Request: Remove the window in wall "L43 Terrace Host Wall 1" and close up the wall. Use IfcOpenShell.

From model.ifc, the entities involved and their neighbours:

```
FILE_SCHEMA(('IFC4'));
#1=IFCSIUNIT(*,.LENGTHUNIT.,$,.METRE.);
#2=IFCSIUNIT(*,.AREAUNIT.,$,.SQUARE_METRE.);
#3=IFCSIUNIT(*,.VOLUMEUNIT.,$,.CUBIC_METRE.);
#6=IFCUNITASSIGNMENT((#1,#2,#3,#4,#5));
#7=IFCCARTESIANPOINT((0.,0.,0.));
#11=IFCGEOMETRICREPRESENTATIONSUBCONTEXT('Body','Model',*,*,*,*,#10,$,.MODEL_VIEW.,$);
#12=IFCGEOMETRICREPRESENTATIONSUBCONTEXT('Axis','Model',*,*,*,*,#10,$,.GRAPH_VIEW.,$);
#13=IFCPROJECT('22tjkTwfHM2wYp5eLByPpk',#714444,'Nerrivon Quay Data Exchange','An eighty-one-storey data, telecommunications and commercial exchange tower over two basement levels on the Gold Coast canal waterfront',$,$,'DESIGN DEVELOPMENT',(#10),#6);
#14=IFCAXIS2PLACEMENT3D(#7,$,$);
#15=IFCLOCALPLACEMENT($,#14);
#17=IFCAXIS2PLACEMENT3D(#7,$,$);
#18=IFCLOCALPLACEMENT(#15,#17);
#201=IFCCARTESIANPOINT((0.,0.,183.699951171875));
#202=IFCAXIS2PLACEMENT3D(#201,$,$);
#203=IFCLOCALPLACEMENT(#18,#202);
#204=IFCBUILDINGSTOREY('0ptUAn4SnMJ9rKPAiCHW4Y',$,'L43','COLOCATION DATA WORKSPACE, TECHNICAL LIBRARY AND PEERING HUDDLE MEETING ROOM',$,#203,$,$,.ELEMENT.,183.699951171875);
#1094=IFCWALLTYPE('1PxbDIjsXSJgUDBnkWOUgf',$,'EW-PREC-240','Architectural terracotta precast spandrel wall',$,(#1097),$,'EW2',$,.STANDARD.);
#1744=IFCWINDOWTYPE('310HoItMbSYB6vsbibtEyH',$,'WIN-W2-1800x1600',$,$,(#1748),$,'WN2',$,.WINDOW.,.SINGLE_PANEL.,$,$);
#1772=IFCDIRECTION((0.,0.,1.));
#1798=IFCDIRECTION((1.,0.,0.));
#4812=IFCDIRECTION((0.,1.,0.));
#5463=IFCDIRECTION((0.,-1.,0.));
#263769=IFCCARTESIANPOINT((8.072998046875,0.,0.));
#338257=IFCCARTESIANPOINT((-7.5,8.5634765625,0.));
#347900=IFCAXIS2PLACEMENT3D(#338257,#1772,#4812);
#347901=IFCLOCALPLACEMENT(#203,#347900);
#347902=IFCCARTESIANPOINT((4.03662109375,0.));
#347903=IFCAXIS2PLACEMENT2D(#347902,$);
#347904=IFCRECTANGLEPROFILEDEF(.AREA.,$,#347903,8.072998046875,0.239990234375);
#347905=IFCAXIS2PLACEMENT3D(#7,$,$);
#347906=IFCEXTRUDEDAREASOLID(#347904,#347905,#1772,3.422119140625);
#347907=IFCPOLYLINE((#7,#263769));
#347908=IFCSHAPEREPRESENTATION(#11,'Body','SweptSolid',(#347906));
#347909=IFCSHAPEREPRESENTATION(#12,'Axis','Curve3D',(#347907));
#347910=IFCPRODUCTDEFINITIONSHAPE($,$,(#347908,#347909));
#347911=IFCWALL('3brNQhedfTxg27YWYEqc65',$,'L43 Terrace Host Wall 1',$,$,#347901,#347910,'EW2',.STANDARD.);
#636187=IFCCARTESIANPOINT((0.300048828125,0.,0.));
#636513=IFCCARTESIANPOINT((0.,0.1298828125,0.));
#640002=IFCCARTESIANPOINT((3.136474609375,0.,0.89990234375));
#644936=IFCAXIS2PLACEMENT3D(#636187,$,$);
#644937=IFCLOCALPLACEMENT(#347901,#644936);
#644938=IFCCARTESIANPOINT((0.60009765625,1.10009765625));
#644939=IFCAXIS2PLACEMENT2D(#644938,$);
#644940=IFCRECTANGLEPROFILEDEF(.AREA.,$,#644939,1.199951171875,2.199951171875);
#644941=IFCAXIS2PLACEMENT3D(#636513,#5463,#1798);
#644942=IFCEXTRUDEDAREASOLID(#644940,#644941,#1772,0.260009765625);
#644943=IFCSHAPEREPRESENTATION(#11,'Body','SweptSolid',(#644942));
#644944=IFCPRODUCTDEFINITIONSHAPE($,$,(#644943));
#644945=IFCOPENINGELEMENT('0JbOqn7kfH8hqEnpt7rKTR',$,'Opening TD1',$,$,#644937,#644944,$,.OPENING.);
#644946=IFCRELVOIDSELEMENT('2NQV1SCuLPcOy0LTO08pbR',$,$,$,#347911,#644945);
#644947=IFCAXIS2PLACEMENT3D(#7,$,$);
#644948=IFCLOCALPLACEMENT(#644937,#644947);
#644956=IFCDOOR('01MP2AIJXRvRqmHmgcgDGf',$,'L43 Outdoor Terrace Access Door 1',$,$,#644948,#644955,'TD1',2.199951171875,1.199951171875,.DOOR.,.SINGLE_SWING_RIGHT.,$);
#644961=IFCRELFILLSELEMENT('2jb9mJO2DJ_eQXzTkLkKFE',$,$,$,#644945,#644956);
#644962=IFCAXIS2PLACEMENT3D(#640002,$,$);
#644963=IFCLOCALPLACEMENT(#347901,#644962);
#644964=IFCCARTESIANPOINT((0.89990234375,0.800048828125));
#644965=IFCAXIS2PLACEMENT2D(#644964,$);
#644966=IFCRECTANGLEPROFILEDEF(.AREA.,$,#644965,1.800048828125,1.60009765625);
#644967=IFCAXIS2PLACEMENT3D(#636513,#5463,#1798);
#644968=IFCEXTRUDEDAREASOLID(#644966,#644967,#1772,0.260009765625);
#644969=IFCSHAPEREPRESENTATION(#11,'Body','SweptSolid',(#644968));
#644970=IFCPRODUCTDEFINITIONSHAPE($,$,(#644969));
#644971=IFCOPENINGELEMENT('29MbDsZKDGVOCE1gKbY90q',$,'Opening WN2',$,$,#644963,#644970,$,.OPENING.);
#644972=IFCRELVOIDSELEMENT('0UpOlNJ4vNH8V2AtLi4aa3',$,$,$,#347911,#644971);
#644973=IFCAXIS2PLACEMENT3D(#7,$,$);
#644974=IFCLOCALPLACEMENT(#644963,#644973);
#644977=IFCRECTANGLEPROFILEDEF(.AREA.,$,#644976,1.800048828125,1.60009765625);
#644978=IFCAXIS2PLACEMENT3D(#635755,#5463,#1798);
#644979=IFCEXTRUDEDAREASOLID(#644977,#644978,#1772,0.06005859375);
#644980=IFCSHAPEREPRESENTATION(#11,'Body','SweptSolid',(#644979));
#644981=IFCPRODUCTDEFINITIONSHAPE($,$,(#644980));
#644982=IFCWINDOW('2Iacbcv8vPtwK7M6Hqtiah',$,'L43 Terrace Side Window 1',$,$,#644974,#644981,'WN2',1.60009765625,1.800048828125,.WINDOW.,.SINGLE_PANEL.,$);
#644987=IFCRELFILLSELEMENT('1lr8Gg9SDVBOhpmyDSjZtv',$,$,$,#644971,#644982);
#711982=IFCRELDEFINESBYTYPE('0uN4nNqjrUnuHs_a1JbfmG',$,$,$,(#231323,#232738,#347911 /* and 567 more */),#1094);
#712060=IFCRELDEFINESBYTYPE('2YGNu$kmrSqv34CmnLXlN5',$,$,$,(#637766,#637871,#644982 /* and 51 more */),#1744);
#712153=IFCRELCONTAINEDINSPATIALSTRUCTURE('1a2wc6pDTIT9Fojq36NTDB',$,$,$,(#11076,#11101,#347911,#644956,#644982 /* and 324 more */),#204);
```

```python
import ifcopenshell
import ifcopenshell.api.feature
import ifcopenshell.api.root
import ifcopenshell.geom
import ifcopenshell.util.shape

model = ifcopenshell.open("model.ifc")
settings = ifcopenshell.geom.settings()


def volume(element):
    """Net volume in cubic metres, openings subtracted."""
    shape = ifcopenshell.geom.create_shape(settings, element)
    return ifcopenshell.util.shape.get_volume(shape.geometry)


window = model.by_guid("2Iacbcv8vPtwK7M6Hqtiah")
opening = window.FillsVoids[0].RelatingOpeningElement
wall = opening.VoidsElements[0].RelatingBuildingElement
before = volume(wall)

ifcopenshell.api.root.remove_product(model, product=window)
ifcopenshell.api.feature.remove_feature(model, feature=opening)

after = volume(wall)

print(f"wall volume {before:.3f} -> {after:.3f} m3")

model.write("model-out.ifc")
```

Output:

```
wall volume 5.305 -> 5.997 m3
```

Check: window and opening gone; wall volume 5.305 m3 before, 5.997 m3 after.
